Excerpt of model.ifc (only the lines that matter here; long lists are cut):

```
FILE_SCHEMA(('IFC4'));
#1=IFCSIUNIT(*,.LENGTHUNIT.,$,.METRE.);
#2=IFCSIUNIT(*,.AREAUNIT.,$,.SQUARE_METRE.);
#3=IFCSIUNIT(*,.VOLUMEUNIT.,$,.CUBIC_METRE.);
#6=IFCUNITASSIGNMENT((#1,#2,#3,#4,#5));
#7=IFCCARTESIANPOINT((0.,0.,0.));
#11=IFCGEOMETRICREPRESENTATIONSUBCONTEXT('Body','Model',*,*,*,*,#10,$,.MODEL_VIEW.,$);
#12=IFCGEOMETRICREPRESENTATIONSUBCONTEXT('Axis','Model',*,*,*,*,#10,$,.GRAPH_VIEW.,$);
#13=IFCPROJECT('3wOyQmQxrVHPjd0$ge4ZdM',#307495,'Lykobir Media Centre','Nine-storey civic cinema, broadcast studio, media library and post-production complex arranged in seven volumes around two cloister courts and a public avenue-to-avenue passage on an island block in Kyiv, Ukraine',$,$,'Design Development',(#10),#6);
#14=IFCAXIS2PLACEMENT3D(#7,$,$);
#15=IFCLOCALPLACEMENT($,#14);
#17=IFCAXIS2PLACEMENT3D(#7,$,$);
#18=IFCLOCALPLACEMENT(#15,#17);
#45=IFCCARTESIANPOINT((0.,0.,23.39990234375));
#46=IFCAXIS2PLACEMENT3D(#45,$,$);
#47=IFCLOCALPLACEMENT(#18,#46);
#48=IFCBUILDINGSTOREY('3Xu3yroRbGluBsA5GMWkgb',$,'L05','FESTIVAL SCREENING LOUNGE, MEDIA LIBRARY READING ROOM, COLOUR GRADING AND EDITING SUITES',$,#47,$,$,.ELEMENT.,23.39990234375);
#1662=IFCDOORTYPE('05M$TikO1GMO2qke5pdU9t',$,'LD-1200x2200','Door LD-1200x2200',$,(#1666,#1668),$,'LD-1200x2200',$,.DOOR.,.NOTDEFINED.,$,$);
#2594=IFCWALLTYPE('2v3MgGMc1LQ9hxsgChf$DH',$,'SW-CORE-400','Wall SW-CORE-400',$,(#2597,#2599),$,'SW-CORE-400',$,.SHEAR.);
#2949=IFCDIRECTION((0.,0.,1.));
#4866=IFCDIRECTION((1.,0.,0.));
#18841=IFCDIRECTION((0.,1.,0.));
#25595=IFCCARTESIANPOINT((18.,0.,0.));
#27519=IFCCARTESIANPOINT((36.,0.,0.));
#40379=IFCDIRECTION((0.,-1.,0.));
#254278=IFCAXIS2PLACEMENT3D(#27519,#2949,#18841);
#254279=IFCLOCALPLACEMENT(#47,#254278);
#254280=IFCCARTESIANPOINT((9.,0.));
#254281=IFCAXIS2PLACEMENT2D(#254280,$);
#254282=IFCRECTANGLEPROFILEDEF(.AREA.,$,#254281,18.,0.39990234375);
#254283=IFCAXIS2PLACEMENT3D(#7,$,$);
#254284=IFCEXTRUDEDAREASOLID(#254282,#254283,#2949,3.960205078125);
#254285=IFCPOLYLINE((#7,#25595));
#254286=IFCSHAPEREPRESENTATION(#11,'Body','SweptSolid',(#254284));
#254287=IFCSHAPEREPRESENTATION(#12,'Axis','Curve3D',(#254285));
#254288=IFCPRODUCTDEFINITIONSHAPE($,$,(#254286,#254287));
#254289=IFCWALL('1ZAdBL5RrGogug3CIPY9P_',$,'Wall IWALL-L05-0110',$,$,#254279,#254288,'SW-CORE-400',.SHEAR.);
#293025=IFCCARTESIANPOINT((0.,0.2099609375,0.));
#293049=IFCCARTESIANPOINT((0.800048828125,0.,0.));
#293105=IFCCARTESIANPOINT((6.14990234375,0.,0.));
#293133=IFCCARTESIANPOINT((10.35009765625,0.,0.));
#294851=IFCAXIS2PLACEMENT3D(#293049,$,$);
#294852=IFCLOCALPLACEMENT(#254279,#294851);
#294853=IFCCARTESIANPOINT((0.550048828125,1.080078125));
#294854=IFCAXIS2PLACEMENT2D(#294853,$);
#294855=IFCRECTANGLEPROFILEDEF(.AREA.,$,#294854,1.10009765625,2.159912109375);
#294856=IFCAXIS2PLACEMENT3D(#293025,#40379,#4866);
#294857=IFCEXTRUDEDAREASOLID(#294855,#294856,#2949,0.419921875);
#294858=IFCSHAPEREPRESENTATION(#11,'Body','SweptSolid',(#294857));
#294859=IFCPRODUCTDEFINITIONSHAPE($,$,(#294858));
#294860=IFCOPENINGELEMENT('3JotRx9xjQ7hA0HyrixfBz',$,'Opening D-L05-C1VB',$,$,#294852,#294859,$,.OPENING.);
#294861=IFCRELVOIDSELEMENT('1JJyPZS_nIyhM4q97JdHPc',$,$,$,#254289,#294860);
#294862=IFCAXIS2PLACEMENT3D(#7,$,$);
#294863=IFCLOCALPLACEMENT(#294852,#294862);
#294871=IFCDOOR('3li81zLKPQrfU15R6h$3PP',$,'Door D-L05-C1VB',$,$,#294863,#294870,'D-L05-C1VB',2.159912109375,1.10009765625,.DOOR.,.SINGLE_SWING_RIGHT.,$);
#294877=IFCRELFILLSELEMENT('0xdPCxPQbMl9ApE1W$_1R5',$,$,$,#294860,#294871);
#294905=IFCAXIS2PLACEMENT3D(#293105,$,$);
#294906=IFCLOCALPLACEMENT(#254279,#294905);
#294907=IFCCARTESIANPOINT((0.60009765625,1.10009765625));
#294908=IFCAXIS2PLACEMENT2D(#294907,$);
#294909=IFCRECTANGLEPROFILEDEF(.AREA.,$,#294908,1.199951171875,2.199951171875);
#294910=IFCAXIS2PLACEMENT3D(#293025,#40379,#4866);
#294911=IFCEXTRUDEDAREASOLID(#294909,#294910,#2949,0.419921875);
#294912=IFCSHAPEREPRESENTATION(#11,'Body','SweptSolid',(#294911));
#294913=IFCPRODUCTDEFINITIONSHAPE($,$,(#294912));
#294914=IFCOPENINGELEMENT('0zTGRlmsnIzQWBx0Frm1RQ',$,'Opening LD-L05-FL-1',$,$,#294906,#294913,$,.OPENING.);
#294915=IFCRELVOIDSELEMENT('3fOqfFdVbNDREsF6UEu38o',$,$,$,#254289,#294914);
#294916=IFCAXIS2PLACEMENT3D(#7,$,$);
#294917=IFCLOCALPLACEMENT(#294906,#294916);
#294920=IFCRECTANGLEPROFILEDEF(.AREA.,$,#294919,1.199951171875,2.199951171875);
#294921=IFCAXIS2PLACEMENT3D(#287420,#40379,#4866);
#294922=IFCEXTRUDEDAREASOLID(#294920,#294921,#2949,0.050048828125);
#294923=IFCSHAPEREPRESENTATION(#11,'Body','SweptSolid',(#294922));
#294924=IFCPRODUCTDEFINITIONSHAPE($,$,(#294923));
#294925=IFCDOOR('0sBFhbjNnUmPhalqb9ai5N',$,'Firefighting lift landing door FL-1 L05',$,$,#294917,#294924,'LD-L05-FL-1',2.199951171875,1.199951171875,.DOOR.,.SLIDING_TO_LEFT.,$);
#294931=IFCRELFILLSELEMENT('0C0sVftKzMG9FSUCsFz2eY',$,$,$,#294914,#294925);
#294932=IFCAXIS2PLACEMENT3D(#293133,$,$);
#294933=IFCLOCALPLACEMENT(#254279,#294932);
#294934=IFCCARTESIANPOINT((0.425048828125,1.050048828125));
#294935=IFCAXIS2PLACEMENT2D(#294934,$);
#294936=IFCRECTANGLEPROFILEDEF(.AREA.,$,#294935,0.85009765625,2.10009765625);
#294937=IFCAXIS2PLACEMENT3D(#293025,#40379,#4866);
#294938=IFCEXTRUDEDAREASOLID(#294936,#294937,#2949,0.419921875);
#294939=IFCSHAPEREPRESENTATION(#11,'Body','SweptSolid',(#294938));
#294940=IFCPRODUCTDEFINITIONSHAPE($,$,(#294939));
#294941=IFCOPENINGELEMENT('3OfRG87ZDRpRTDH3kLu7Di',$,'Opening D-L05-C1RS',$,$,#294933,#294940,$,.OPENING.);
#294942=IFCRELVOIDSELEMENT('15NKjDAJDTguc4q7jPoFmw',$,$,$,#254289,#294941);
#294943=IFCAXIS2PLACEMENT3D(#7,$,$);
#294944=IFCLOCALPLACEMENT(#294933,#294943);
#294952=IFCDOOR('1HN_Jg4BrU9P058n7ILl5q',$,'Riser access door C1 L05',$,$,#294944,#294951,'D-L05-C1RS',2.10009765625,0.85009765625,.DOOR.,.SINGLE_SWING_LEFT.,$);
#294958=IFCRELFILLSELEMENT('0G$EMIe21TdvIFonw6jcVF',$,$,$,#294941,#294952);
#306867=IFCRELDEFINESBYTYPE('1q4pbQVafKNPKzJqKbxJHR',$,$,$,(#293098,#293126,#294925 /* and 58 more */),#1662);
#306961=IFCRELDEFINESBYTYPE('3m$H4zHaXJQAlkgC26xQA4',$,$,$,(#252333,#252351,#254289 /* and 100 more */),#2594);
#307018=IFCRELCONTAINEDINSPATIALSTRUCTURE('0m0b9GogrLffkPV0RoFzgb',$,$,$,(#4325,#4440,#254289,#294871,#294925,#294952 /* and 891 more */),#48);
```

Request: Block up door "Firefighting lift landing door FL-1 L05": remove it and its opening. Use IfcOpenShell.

```python
import ifcopenshell
import ifcopenshell.api.feature
import ifcopenshell.api.root
import ifcopenshell.geom
import ifcopenshell.util.shape

model = ifcopenshell.open("model.ifc")
settings = ifcopenshell.geom.settings()


def volume(element):
    """Net volume in cubic metres, openings subtracted."""
    shape = ifcopenshell.geom.create_shape(settings, element)
    return ifcopenshell.util.shape.get_volume(shape.geometry)


door = model.by_id(294925)
opening = door.FillsVoids[0].RelatingOpeningElement
wall = opening.VoidsElements[0].RelatingBuildingElement
before = volume(wall)

ifcopenshell.api.root.remove_product(model, product=door)
ifcopenshell.api.feature.remove_feature(model, feature=opening)

after = volume(wall)

print(f"wall volume {before:.3f} -> {after:.3f} m3")

model.write("model_rev.ifc")
```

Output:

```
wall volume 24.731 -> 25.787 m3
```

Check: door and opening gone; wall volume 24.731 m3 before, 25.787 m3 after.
